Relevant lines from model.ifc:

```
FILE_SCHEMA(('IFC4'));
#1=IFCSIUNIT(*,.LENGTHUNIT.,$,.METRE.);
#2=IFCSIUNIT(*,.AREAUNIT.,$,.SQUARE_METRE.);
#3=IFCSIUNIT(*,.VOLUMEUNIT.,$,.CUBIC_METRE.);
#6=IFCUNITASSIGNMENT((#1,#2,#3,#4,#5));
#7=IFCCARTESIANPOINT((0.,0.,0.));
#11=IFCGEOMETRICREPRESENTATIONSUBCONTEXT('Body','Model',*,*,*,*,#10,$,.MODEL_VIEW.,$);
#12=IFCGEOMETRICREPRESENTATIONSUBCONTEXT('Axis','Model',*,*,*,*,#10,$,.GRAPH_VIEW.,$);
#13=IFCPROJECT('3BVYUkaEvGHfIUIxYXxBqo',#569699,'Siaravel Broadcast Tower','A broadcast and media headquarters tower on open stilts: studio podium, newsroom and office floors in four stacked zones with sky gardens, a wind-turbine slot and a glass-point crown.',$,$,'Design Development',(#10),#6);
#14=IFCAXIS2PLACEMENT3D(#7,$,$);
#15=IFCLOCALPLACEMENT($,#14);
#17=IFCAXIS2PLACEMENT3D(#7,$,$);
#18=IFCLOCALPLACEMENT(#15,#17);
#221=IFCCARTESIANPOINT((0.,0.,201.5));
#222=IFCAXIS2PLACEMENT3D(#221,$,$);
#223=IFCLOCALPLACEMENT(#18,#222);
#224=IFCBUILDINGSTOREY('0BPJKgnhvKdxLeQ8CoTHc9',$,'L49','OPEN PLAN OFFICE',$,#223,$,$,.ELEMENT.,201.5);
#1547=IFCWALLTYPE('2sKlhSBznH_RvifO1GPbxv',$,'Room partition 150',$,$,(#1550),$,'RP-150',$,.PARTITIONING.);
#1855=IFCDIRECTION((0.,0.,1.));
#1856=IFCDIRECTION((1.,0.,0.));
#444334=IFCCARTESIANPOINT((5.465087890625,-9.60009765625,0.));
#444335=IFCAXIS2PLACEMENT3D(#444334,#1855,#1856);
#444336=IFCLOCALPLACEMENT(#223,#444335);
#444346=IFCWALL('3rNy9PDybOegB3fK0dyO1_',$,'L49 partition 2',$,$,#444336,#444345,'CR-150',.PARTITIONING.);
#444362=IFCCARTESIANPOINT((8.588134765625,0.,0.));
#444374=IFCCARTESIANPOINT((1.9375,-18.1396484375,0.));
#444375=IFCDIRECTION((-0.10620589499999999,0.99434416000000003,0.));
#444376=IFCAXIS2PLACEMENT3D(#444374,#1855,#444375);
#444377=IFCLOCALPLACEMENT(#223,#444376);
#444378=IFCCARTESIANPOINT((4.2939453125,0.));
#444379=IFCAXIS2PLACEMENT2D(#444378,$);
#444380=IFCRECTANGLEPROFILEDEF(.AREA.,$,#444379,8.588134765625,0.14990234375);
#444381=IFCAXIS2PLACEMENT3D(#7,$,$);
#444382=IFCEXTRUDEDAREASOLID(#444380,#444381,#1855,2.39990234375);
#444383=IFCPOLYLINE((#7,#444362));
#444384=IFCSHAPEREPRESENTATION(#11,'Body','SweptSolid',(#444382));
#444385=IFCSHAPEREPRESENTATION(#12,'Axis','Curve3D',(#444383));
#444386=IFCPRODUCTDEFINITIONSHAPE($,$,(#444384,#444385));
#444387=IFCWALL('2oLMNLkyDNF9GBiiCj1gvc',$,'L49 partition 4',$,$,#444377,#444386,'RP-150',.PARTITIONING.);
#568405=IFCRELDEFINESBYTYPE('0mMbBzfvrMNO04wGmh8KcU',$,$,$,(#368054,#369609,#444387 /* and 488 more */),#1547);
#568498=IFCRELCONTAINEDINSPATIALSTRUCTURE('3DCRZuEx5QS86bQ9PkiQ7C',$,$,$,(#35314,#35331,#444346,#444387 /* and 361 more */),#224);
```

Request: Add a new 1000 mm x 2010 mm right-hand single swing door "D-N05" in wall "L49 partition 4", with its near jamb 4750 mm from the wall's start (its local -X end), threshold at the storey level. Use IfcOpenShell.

```python
import numpy as np
import ifcopenshell
import ifcopenshell.api.feature
import ifcopenshell.api.geometry
import ifcopenshell.api.root
import ifcopenshell.api.spatial
import ifcopenshell.geom
import ifcopenshell.util.element
import ifcopenshell.util.placement
import ifcopenshell.util.representation
import ifcopenshell.util.shape
import ifcopenshell.util.unit

model = ifcopenshell.open("model.ifc")
unit_scale = ifcopenshell.util.unit.calculate_unit_scale(model)
settings = ifcopenshell.geom.settings()


def volume(element):
    """Net volume in cubic metres, openings subtracted."""
    shape = ifcopenshell.geom.create_shape(settings, element)
    return ifcopenshell.util.shape.get_volume(shape.geometry)


wall = model.by_id(444387)
storey = ifcopenshell.util.element.get_container(wall, ifc_class="IfcBuildingStorey")
context = ifcopenshell.util.representation.get_context(model, "Model", "Body", "MODEL_VIEW")
before = volume(wall)

width, height, from_end, sill = 1, 2.01, 4.75, 0.0  # metres

# The wall runs along its own X axis, and the end named is its -X end.
wall_shape = ifcopenshell.geom.create_shape(settings, wall)
x, y, z = ifcopenshell.util.shape.get_vertices(wall_shape.geometry).T
start = x.min() + from_end
face, thickness = float(y.min()), float(y.max() - y.min())
wall_matrix = ifcopenshell.util.placement.get_local_placement(wall.ObjectPlacement)
level = ifcopenshell.util.placement.get_local_placement(storey.ObjectPlacement)[2, 3]


def in_wall(x, y):
    """Placement at x, y metres in the wall's axes, at sill height."""
    matrix = wall_matrix.copy()
    matrix[:, 3] = wall_matrix @ np.array([x / unit_scale, y / unit_scale, 0.0, 1.0])
    matrix[2, 3] = level + sill / unit_scale
    return matrix


# Opening: a box that overshoots both wall faces by 50 mm.
opening = ifcopenshell.api.root.create_entity(model, ifc_class="IfcOpeningElement", predefined_type="OPENING")
box = ifcopenshell.api.geometry.add_wall_representation(
    model, context=context, length=width, height=height, thickness=thickness + 0.1
)
ifcopenshell.api.geometry.assign_representation(model, product=opening, representation=box)
ifcopenshell.api.geometry.edit_object_placement(model, product=opening, matrix=in_wall(start, face - 0.05), is_si=False)
ifcopenshell.api.feature.add_feature(model, feature=opening, element=wall)

door = ifcopenshell.api.root.create_entity(model, ifc_class="IfcDoor", name="D-N05", predefined_type="DOOR")
door.OverallWidth, door.OverallHeight = width / unit_scale, height / unit_scale
door.OperationType = "SINGLE_SWING_RIGHT"
body = ifcopenshell.api.geometry.add_door_representation(
    model,
    context=context,
    overall_width=door.OverallWidth,
    overall_height=door.OverallHeight,
    operation_type="SINGLE_SWING_RIGHT",
    lining_properties={"LiningDepth": thickness / unit_scale, "ThresholdDepth": thickness / unit_scale},
)
ifcopenshell.api.geometry.assign_representation(model, product=door, representation=body)
ifcopenshell.api.spatial.assign_container(model, products=[door], relating_structure=storey)
ifcopenshell.api.feature.add_filling(model, opening=opening, element=door)

# The lining spans the wall, so the door starts at the wall face.
ifcopenshell.api.geometry.edit_object_placement(model, product=door, matrix=in_wall(start, face), is_si=False)

after = volume(wall)

print(f"wall volume {before:.3f} -> {after:.3f} m3")

model.write("model_updated.ifc")
```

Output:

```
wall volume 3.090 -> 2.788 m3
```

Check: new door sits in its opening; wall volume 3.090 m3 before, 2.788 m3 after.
